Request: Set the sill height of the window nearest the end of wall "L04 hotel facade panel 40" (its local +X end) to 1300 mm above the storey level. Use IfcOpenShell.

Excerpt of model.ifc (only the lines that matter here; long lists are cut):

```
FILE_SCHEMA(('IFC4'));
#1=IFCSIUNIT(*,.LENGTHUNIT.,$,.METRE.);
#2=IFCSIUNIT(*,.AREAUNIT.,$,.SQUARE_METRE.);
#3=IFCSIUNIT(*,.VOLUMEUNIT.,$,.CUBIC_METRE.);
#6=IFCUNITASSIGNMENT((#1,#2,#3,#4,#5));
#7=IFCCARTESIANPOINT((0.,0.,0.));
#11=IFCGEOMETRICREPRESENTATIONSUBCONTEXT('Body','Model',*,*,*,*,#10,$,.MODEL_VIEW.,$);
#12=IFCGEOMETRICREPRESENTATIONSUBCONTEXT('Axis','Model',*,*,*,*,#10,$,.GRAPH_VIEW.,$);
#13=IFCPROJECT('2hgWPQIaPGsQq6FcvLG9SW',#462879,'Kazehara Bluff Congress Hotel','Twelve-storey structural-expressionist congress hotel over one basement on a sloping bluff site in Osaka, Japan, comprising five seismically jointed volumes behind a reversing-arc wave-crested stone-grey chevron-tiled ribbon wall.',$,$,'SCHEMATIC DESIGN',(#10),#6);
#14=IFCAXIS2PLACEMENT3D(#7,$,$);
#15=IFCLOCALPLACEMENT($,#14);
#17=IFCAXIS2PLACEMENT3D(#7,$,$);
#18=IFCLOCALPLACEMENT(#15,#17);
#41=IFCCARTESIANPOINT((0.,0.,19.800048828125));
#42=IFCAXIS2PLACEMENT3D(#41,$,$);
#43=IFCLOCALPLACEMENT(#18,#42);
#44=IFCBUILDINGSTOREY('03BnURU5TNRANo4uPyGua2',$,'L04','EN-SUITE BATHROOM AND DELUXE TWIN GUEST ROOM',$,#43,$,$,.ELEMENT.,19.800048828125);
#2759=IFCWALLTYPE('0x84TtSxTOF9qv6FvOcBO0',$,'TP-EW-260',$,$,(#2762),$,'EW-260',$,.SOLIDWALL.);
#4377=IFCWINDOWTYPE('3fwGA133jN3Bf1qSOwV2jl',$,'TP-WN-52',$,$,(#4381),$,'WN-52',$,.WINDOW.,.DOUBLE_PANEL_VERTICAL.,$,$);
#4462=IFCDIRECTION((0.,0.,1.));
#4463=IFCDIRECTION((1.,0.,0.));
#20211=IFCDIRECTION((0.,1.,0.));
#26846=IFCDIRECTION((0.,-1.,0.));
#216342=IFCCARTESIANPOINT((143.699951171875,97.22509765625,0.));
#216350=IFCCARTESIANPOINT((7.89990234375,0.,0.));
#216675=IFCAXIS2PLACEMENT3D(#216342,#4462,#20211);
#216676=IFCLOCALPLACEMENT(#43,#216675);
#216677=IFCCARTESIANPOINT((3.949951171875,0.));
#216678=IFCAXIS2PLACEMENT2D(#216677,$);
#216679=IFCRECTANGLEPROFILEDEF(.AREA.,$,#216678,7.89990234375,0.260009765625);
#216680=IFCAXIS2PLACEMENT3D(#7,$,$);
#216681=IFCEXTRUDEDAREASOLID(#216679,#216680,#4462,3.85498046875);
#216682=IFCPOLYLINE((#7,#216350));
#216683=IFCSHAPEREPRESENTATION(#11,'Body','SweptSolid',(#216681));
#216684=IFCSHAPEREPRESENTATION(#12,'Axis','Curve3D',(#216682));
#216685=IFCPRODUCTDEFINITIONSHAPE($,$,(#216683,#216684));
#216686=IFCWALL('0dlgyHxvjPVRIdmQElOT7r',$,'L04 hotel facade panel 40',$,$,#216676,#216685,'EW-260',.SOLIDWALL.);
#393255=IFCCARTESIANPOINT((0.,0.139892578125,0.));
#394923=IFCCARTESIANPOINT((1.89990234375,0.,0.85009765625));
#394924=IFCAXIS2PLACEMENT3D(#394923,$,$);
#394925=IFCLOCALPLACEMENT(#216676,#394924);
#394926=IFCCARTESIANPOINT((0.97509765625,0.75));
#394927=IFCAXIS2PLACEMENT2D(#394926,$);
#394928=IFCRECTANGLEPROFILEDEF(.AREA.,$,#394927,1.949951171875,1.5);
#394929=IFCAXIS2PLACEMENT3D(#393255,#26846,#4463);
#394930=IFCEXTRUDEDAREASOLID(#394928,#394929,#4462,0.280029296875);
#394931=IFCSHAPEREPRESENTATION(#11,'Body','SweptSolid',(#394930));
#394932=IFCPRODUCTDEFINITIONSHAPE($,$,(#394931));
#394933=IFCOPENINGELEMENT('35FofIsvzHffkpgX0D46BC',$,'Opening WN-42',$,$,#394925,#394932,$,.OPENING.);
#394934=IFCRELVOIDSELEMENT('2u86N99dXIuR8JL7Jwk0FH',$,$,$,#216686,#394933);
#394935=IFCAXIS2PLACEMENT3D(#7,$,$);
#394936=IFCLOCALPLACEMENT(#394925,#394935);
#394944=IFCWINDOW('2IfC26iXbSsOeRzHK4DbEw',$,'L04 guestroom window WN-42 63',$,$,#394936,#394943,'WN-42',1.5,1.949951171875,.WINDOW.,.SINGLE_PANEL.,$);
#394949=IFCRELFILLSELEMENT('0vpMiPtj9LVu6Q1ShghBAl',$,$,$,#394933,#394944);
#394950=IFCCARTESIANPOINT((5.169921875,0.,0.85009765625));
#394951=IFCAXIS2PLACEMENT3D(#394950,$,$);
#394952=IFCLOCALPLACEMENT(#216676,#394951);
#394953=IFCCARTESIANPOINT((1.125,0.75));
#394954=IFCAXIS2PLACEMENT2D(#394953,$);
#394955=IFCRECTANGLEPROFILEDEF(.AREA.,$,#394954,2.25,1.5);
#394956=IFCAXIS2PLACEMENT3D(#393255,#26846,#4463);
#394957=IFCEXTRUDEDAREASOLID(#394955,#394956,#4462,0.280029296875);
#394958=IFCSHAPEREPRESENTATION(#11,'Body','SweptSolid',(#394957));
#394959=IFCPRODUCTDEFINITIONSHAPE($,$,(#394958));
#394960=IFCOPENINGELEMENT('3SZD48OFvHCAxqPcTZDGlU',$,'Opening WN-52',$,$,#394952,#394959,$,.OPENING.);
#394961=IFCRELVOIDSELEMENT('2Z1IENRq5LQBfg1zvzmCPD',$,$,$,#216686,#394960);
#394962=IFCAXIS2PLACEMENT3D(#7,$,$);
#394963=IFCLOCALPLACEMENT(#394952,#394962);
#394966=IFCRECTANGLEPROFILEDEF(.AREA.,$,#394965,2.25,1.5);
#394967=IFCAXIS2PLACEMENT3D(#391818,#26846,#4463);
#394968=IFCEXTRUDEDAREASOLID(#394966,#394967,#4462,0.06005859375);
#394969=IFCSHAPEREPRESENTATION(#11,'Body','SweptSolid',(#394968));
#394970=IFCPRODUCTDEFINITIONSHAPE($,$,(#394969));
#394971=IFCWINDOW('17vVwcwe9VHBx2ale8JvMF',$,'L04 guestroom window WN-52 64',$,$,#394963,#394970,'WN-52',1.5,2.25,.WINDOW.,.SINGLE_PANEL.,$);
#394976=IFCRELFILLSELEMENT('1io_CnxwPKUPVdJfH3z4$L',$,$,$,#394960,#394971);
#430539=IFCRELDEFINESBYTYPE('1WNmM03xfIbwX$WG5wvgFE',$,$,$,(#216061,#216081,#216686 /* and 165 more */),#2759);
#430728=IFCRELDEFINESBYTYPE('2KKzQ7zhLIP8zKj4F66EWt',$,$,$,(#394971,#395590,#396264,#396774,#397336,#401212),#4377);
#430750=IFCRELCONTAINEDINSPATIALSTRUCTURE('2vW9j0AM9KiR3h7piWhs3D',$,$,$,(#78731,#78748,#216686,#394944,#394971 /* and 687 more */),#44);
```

```python
import numpy as np
import ifcopenshell
import ifcopenshell.api.geometry
import ifcopenshell.geom
import ifcopenshell.util.element
import ifcopenshell.util.placement
import ifcopenshell.util.shape
import ifcopenshell.util.unit

model = ifcopenshell.open("model.ifc")
unit_scale = ifcopenshell.util.unit.calculate_unit_scale(model)

window = model.by_guid("17vVwcwe9VHBx2ale8JvMF")
opening = window.FillsVoids[0].RelatingOpeningElement
storey = ifcopenshell.util.element.get_container(window, ifc_class="IfcBuildingStorey")
level = ifcopenshell.util.placement.get_local_placement(storey.ObjectPlacement)[2, 3]

# The opening's origin need not be at the sill, so measure its lowest point.
shape = ifcopenshell.geom.create_shape(ifcopenshell.geom.settings(), opening)
bottom = ifcopenshell.util.shape.get_shape_bottom_elevation(shape, shape.geometry) / unit_scale
dz = level + 1.3 / unit_scale - bottom

shift = np.array([0.0, 0.0, dz])
# The window is placed relative to its opening, so it follows when the opening moves.
matrix = ifcopenshell.util.placement.get_local_placement(opening.ObjectPlacement)
matrix[:3, 3] += shift
ifcopenshell.api.geometry.edit_object_placement(
    model, product=opening, matrix=matrix, is_si=False, should_transform_children=True
)

print(f"moved by {dz * unit_scale:+.3f} m")

model.write("model_edited.ifc")
```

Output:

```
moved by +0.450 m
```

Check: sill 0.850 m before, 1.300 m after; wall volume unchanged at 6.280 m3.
